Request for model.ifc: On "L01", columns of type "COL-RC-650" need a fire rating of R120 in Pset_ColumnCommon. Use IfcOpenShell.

First a look at what the model holds.

```python
import ifcopenshell
import ifcopenshell.util.element

model = ifcopenshell.open("model.ifc")
print(model.schema)
storey = next(s for s in model.by_type("IfcBuildingStorey") if s.Name == "L01")
columns = [e for e in ifcopenshell.util.element.get_decomposition(storey) if e.is_a("IfcColumn")]
seen = {}
for e in columns:
    element_type = ifcopenshell.util.element.get_type(e)
    key = (element_type.Name if element_type != e and element_type else None, ifcopenshell.util.element.get_pset(e, "Pset_ColumnCommon", "FireRating"))
    seen[key] = seen.get(key, 0) + 1
for (name, value), count in sorted(seen.items(), key=str):
    print(count, "x", name, "|", value)
```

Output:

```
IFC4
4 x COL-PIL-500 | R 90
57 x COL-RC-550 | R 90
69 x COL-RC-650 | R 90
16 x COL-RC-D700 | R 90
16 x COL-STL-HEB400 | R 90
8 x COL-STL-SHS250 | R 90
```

```python
import ifcopenshell
import ifcopenshell.api.pset
import ifcopenshell.util.element

model = ifcopenshell.open("model.ifc")

storey = next(s for s in model.by_type("IfcBuildingStorey") if s.Name == "L01")
columns = [e for e in ifcopenshell.util.element.get_decomposition(storey) if e.is_a("IfcColumn")]

count = 0
for e in columns:
    element_type = ifcopenshell.util.element.get_type(e)
    if element_type in (None, e) or element_type.Name != "COL-RC-650":
        continue
    # add_pset returns the element's existing set when there is one.
    pset = ifcopenshell.api.pset.add_pset(model, product=e, name="Pset_ColumnCommon")
    ifcopenshell.api.pset.edit_pset(model, pset=pset, properties={"FireRating": "R120"})
    count += 1

print(count, "columns updated")

model.write("model-out.ifc")
```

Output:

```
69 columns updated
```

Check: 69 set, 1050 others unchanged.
